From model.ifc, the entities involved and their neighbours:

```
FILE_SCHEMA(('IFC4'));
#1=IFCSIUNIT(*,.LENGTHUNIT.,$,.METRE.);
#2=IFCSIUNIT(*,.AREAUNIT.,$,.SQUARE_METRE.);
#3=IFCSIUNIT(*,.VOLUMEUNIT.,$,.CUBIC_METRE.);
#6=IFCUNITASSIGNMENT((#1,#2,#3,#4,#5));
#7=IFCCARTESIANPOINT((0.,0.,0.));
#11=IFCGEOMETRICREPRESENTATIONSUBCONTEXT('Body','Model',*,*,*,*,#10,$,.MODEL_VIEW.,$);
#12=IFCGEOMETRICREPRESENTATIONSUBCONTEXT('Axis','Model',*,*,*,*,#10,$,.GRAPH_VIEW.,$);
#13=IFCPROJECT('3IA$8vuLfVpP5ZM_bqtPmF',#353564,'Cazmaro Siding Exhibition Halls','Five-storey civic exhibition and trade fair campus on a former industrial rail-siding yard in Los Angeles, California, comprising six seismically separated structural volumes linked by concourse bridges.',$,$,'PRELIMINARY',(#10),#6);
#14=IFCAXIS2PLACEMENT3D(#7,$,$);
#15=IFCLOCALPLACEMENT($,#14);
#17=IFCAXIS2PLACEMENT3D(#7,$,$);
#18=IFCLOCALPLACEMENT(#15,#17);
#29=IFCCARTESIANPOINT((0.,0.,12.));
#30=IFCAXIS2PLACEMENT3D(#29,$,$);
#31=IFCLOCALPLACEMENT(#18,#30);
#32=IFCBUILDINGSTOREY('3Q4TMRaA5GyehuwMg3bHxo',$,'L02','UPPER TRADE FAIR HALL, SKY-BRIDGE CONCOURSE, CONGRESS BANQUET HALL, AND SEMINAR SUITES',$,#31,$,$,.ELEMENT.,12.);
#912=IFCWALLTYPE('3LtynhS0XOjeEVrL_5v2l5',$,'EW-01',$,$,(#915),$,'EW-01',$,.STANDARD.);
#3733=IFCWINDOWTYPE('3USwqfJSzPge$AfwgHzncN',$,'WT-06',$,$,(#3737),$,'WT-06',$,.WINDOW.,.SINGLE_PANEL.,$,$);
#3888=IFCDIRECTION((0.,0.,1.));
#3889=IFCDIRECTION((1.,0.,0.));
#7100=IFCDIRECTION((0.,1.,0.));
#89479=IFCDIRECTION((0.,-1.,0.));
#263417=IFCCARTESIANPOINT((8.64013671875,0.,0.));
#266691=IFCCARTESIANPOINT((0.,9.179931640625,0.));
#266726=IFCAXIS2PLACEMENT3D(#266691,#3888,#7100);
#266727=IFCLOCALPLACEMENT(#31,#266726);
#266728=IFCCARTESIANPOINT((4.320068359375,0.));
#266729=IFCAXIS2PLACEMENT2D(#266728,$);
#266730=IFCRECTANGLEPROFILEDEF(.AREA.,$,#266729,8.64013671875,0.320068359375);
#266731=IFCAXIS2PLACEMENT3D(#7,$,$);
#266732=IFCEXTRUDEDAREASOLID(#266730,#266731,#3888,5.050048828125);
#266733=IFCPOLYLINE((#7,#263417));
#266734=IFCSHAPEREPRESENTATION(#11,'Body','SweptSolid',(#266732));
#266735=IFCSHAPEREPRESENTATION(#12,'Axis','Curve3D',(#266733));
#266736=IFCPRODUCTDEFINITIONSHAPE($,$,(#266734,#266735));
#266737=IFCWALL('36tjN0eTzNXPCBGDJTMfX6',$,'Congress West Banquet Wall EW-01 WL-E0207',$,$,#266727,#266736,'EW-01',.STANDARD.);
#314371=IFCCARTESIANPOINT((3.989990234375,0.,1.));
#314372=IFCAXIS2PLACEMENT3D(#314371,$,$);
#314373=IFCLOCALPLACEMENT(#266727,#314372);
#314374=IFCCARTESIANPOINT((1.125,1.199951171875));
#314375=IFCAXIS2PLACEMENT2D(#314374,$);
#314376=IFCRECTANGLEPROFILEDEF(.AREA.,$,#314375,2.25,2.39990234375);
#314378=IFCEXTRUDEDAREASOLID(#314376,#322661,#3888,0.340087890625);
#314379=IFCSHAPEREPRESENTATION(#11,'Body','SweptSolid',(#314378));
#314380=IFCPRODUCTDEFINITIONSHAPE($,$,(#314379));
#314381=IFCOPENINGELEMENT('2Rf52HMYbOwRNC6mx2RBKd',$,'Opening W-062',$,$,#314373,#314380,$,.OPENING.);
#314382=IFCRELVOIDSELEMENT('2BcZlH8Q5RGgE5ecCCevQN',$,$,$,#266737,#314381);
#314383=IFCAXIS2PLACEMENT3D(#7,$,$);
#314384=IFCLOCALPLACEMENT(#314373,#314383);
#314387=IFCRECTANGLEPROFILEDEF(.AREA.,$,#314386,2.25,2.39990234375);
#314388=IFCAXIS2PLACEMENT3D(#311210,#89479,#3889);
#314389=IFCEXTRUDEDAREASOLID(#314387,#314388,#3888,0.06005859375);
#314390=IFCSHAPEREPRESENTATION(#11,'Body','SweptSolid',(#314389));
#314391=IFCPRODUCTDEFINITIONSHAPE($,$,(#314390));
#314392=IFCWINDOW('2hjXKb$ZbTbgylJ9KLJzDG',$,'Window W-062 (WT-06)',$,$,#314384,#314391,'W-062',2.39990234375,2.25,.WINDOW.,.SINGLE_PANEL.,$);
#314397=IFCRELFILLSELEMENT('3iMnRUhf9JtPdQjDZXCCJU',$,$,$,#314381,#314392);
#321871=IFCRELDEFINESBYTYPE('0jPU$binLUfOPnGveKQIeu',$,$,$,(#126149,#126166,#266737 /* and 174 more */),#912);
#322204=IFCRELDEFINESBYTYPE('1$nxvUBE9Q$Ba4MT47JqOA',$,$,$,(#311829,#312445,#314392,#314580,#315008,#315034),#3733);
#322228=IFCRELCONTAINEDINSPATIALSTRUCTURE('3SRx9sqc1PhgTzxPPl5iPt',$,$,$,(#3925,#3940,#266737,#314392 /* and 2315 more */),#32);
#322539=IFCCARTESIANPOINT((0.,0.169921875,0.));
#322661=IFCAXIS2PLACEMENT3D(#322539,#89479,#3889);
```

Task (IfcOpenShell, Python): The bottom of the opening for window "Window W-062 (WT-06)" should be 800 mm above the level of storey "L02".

```python
import numpy as np
import ifcopenshell
import ifcopenshell.api.geometry
import ifcopenshell.geom
import ifcopenshell.util.element
import ifcopenshell.util.placement
import ifcopenshell.util.shape
import ifcopenshell.util.unit

model = ifcopenshell.open("model.ifc")
unit_scale = ifcopenshell.util.unit.calculate_unit_scale(model)

window = model.by_id(314392)
opening = window.FillsVoids[0].RelatingOpeningElement
storey = ifcopenshell.util.element.get_container(window, ifc_class="IfcBuildingStorey")
level = ifcopenshell.util.placement.get_local_placement(storey.ObjectPlacement)[2, 3]

# The opening's origin need not be at the sill, so measure its lowest point.
shape = ifcopenshell.geom.create_shape(ifcopenshell.geom.settings(), opening)
bottom = ifcopenshell.util.shape.get_shape_bottom_elevation(shape, shape.geometry) / unit_scale
dz = level + 0.8 / unit_scale - bottom

shift = np.array([0.0, 0.0, dz])
# The window is placed relative to its opening, so it follows when the opening moves.
matrix = ifcopenshell.util.placement.get_local_placement(opening.ObjectPlacement)
matrix[:3, 3] += shift
ifcopenshell.api.geometry.edit_object_placement(
    model, product=opening, matrix=matrix, is_si=False, should_transform_children=True
)

print(f"moved by {dz * unit_scale:+.3f} m")

model.write("model_edited.ifc")
```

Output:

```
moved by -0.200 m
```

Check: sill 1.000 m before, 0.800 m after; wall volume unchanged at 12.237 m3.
